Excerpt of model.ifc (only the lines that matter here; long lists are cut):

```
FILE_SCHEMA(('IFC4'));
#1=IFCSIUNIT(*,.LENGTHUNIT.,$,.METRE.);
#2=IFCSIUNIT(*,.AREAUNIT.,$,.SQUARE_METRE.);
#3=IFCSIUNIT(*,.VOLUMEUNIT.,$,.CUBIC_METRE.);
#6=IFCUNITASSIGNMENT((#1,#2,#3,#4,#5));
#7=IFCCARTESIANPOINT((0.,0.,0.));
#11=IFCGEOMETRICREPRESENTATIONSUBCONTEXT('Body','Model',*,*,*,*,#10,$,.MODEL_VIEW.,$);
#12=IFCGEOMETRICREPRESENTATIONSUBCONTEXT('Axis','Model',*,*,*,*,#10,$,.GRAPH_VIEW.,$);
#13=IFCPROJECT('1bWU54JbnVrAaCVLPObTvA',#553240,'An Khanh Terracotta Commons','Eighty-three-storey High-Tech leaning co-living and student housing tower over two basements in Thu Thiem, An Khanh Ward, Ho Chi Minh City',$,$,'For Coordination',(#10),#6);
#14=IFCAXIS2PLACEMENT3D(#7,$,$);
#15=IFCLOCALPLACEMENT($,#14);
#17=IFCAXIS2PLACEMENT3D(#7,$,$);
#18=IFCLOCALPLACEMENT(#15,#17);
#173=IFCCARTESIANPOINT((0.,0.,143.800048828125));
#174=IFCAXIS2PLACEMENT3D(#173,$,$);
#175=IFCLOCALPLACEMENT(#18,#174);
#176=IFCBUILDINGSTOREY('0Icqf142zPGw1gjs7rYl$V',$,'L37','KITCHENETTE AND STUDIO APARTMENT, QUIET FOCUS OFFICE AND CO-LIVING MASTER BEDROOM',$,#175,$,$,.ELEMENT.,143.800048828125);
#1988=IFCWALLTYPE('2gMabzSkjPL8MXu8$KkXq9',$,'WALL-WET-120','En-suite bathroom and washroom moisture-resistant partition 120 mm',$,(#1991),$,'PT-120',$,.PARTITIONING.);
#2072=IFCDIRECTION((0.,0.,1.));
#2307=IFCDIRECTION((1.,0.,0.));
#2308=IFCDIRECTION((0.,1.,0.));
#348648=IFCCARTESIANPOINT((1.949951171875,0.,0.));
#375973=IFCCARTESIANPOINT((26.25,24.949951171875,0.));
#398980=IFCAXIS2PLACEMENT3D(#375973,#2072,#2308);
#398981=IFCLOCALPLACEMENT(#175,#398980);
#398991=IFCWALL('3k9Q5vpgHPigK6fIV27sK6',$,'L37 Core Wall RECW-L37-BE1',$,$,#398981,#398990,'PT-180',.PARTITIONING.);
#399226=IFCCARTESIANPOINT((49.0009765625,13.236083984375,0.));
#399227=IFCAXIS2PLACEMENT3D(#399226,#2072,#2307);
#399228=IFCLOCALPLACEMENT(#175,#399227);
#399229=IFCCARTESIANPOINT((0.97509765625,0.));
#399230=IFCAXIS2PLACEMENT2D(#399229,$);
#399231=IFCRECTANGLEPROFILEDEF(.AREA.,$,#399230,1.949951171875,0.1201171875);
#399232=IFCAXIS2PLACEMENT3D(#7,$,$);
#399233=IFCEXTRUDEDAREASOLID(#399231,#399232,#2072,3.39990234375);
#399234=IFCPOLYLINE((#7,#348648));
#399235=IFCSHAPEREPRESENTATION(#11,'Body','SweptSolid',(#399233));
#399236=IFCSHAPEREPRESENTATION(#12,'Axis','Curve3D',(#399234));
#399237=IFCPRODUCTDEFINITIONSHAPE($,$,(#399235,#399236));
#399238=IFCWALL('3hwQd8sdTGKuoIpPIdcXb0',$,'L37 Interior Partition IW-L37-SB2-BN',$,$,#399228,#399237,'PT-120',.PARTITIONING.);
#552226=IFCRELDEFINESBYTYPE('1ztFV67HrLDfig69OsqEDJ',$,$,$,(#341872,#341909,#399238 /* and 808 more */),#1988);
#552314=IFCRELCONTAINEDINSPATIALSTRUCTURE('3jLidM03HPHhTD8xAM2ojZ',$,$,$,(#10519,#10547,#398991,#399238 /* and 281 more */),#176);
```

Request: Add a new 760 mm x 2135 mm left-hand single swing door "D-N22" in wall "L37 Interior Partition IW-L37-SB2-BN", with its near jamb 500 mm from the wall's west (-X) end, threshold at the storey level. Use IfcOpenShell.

```python
import numpy as np
import ifcopenshell
import ifcopenshell.api.feature
import ifcopenshell.api.geometry
import ifcopenshell.api.root
import ifcopenshell.api.spatial
import ifcopenshell.geom
import ifcopenshell.util.element
import ifcopenshell.util.placement
import ifcopenshell.util.representation
import ifcopenshell.util.shape
import ifcopenshell.util.unit

model = ifcopenshell.open("model.ifc")
unit_scale = ifcopenshell.util.unit.calculate_unit_scale(model)
settings = ifcopenshell.geom.settings()


def volume(element):
    """Net volume in cubic metres, openings subtracted."""
    shape = ifcopenshell.geom.create_shape(settings, element)
    return ifcopenshell.util.shape.get_volume(shape.geometry)


wall = model.by_guid("3hwQd8sdTGKuoIpPIdcXb0")
storey = ifcopenshell.util.element.get_container(wall, ifc_class="IfcBuildingStorey")
context = ifcopenshell.util.representation.get_context(model, "Model", "Body", "MODEL_VIEW")
before = volume(wall)

width, height, from_end, sill = 0.76, 2.135, 0.5, 0.0  # metres

# The wall runs along its own X axis, and the end named is its -X end.
wall_shape = ifcopenshell.geom.create_shape(settings, wall)
x, y, z = ifcopenshell.util.shape.get_vertices(wall_shape.geometry).T
start = x.min() + from_end
face, thickness = float(y.min()), float(y.max() - y.min())
wall_matrix = ifcopenshell.util.placement.get_local_placement(wall.ObjectPlacement)
level = ifcopenshell.util.placement.get_local_placement(storey.ObjectPlacement)[2, 3]


def in_wall(x, y):
    """Placement at x, y metres in the wall's axes, at sill height."""
    matrix = wall_matrix.copy()
    matrix[:, 3] = wall_matrix @ np.array([x / unit_scale, y / unit_scale, 0.0, 1.0])
    matrix[2, 3] = level + sill / unit_scale
    return matrix


# Opening: a box that overshoots both wall faces by 50 mm.
opening = ifcopenshell.api.root.create_entity(model, ifc_class="IfcOpeningElement", predefined_type="OPENING")
box = ifcopenshell.api.geometry.add_wall_representation(
    model, context=context, length=width, height=height, thickness=thickness + 0.1
)
ifcopenshell.api.geometry.assign_representation(model, product=opening, representation=box)
ifcopenshell.api.geometry.edit_object_placement(model, product=opening, matrix=in_wall(start, face - 0.05), is_si=False)
ifcopenshell.api.feature.add_feature(model, feature=opening, element=wall)

door = ifcopenshell.api.root.create_entity(model, ifc_class="IfcDoor", name="D-N22", predefined_type="DOOR")
door.OverallWidth, door.OverallHeight = width / unit_scale, height / unit_scale
door.OperationType = "SINGLE_SWING_LEFT"
body = ifcopenshell.api.geometry.add_door_representation(
    model,
    context=context,
    overall_width=door.OverallWidth,
    overall_height=door.OverallHeight,
    operation_type="SINGLE_SWING_LEFT",
    lining_properties={"LiningDepth": thickness / unit_scale, "ThresholdDepth": thickness / unit_scale},
)
ifcopenshell.api.geometry.assign_representation(model, product=door, representation=body)
ifcopenshell.api.spatial.assign_container(model, products=[door], relating_structure=storey)
ifcopenshell.api.feature.add_filling(model, opening=opening, element=door)

# The lining spans the wall, so the door starts at the wall face.
ifcopenshell.api.geometry.edit_object_placement(model, product=door, matrix=in_wall(start, face), is_si=False)

after = volume(wall)

print(f"wall volume {before:.3f} -> {after:.3f} m3")

model.write("model_edited.ifc")
```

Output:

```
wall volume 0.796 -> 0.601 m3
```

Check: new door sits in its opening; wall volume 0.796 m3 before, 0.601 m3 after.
